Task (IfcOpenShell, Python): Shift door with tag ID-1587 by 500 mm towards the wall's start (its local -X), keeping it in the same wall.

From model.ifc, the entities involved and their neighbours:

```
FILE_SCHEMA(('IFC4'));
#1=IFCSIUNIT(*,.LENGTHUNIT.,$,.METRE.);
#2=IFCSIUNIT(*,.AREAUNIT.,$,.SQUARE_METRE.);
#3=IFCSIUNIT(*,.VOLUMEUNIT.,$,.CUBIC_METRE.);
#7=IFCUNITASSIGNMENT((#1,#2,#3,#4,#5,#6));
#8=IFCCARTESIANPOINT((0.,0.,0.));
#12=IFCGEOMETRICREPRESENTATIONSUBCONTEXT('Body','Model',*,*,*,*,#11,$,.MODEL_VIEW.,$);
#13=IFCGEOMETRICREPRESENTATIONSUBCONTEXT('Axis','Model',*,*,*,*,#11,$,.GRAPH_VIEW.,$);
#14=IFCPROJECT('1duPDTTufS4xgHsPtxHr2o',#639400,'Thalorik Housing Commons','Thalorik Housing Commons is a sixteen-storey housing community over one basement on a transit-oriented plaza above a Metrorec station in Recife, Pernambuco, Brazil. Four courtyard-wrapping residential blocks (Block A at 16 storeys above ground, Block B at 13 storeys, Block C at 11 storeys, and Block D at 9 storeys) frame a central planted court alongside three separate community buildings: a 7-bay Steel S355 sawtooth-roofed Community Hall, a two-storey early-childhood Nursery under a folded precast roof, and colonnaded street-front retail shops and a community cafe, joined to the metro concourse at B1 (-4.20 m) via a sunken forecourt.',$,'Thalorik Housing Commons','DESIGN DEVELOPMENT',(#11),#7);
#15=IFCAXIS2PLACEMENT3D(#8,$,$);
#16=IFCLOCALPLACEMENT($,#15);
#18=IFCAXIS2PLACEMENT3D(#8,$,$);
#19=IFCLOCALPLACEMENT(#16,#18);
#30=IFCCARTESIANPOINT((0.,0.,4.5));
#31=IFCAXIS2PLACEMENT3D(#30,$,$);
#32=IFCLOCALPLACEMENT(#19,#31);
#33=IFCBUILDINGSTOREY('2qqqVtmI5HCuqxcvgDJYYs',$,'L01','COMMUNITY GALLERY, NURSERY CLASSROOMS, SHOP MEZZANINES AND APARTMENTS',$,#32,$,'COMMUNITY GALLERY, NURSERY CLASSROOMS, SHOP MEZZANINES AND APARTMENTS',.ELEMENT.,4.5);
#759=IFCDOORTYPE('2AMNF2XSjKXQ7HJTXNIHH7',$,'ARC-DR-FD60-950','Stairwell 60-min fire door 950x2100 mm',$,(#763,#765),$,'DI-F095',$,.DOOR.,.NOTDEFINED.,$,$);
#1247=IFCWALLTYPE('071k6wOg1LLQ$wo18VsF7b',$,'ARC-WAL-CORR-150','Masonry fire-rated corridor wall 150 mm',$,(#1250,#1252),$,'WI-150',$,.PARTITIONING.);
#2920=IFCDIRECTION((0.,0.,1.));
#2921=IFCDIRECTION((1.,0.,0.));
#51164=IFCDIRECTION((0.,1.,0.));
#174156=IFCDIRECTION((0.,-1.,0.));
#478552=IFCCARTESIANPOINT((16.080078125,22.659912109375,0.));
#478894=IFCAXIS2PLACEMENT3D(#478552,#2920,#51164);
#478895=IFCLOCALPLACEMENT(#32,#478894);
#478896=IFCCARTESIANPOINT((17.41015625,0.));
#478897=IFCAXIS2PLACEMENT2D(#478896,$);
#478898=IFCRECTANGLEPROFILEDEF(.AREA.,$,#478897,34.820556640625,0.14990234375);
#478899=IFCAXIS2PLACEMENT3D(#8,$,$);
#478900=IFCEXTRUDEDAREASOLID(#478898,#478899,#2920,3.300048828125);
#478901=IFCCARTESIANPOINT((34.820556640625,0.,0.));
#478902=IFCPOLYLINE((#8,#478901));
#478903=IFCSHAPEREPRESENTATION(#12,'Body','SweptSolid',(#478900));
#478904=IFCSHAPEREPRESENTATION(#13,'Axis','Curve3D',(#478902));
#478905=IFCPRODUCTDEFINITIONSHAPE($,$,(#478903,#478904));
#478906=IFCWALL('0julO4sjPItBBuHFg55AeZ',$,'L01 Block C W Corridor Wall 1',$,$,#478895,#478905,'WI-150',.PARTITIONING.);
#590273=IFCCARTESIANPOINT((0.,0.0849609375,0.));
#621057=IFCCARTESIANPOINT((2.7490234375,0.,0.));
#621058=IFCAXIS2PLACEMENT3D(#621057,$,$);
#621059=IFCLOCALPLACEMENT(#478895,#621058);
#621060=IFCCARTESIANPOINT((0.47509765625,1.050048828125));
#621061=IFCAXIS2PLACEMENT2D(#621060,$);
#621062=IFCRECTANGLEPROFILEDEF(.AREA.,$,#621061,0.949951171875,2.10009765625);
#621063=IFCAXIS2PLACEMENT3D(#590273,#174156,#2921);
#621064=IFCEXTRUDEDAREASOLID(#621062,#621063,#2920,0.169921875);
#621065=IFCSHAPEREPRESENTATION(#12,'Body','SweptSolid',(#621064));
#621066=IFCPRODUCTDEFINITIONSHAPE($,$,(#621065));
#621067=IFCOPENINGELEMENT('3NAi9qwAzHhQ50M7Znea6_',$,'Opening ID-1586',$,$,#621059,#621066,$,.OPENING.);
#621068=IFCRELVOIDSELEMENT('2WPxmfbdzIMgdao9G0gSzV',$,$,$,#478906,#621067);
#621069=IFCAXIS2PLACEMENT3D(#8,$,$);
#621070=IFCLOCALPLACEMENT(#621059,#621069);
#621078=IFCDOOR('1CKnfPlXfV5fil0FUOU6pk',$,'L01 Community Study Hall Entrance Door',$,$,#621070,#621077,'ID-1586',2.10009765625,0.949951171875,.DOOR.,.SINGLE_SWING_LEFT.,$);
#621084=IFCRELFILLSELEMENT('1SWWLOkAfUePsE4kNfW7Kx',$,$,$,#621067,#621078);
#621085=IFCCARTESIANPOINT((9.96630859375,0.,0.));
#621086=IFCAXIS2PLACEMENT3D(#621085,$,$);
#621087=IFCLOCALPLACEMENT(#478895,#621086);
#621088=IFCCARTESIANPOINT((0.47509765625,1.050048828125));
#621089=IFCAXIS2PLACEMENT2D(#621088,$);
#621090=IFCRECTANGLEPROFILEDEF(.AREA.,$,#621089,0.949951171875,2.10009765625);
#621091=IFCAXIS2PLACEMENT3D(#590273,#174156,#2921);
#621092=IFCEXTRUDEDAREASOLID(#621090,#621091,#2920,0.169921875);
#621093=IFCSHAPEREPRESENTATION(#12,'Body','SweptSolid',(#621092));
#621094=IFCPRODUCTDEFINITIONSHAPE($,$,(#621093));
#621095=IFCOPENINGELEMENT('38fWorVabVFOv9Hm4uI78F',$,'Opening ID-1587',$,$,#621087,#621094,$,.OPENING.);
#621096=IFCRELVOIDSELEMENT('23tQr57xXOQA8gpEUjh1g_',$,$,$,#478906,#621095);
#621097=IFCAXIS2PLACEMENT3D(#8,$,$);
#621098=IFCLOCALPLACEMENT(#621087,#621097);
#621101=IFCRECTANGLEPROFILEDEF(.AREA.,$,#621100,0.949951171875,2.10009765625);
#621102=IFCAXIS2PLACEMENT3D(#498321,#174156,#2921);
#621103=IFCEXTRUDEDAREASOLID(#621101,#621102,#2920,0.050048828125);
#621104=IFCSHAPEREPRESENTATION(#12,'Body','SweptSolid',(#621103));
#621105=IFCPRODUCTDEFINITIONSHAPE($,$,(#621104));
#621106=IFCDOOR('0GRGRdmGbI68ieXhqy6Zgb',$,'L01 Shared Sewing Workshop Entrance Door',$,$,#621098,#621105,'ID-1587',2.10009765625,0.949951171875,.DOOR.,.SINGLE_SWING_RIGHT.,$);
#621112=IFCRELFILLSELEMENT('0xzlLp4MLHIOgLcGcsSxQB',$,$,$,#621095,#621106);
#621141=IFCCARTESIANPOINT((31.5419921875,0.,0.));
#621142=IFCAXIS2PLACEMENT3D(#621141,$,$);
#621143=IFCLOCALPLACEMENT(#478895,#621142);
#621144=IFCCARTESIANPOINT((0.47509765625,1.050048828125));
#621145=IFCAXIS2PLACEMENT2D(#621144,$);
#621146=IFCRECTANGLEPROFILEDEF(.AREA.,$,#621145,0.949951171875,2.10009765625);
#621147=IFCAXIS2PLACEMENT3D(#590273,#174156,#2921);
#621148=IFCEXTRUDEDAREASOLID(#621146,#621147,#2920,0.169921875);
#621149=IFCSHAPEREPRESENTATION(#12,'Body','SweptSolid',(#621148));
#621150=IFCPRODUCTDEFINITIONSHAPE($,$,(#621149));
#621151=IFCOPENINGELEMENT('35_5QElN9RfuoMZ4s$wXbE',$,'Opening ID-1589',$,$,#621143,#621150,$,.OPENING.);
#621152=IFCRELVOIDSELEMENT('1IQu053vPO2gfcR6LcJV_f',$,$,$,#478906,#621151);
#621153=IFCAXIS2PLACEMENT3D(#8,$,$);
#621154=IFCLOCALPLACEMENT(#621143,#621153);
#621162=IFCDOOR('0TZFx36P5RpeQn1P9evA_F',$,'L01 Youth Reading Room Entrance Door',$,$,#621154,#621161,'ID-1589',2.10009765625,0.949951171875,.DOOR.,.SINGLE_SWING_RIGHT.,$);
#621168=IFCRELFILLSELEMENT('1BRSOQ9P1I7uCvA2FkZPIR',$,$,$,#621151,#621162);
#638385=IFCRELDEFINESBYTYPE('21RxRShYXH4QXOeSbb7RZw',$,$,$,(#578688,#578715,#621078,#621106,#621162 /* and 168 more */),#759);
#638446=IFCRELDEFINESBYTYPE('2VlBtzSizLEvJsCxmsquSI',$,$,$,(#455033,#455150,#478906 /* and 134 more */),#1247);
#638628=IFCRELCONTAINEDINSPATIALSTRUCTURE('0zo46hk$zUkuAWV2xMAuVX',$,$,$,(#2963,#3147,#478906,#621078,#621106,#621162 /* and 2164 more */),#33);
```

```python
import ifcopenshell
import ifcopenshell.api.geometry
import ifcopenshell.util.placement
import ifcopenshell.util.unit

model = ifcopenshell.open("model.ifc")
unit_scale = ifcopenshell.util.unit.calculate_unit_scale(model)

door = model.by_id(621106)
opening = door.FillsVoids[0].RelatingOpeningElement
wall = opening.VoidsElements[0].RelatingBuildingElement

wall_matrix = ifcopenshell.util.placement.get_local_placement(wall.ObjectPlacement)
shift = wall_matrix[:3, 0] * -0.5 / unit_scale
before = ifcopenshell.util.placement.get_local_placement(door.ObjectPlacement)[:3, 3].copy()

# The door is placed relative to its opening, so it follows when the opening moves.
matrix = ifcopenshell.util.placement.get_local_placement(opening.ObjectPlacement)
matrix[:3, 3] += shift
ifcopenshell.api.geometry.edit_object_placement(
    model, product=opening, matrix=matrix, is_si=False, should_transform_children=True
)

after = ifcopenshell.util.placement.get_local_placement(door.ObjectPlacement)[:3, 3]
print("door moved by", (after - before).round(3) + 0.0)

model.write("model_rev.ifc")
```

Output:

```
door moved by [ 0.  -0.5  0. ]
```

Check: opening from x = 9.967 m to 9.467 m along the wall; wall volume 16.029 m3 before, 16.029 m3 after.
